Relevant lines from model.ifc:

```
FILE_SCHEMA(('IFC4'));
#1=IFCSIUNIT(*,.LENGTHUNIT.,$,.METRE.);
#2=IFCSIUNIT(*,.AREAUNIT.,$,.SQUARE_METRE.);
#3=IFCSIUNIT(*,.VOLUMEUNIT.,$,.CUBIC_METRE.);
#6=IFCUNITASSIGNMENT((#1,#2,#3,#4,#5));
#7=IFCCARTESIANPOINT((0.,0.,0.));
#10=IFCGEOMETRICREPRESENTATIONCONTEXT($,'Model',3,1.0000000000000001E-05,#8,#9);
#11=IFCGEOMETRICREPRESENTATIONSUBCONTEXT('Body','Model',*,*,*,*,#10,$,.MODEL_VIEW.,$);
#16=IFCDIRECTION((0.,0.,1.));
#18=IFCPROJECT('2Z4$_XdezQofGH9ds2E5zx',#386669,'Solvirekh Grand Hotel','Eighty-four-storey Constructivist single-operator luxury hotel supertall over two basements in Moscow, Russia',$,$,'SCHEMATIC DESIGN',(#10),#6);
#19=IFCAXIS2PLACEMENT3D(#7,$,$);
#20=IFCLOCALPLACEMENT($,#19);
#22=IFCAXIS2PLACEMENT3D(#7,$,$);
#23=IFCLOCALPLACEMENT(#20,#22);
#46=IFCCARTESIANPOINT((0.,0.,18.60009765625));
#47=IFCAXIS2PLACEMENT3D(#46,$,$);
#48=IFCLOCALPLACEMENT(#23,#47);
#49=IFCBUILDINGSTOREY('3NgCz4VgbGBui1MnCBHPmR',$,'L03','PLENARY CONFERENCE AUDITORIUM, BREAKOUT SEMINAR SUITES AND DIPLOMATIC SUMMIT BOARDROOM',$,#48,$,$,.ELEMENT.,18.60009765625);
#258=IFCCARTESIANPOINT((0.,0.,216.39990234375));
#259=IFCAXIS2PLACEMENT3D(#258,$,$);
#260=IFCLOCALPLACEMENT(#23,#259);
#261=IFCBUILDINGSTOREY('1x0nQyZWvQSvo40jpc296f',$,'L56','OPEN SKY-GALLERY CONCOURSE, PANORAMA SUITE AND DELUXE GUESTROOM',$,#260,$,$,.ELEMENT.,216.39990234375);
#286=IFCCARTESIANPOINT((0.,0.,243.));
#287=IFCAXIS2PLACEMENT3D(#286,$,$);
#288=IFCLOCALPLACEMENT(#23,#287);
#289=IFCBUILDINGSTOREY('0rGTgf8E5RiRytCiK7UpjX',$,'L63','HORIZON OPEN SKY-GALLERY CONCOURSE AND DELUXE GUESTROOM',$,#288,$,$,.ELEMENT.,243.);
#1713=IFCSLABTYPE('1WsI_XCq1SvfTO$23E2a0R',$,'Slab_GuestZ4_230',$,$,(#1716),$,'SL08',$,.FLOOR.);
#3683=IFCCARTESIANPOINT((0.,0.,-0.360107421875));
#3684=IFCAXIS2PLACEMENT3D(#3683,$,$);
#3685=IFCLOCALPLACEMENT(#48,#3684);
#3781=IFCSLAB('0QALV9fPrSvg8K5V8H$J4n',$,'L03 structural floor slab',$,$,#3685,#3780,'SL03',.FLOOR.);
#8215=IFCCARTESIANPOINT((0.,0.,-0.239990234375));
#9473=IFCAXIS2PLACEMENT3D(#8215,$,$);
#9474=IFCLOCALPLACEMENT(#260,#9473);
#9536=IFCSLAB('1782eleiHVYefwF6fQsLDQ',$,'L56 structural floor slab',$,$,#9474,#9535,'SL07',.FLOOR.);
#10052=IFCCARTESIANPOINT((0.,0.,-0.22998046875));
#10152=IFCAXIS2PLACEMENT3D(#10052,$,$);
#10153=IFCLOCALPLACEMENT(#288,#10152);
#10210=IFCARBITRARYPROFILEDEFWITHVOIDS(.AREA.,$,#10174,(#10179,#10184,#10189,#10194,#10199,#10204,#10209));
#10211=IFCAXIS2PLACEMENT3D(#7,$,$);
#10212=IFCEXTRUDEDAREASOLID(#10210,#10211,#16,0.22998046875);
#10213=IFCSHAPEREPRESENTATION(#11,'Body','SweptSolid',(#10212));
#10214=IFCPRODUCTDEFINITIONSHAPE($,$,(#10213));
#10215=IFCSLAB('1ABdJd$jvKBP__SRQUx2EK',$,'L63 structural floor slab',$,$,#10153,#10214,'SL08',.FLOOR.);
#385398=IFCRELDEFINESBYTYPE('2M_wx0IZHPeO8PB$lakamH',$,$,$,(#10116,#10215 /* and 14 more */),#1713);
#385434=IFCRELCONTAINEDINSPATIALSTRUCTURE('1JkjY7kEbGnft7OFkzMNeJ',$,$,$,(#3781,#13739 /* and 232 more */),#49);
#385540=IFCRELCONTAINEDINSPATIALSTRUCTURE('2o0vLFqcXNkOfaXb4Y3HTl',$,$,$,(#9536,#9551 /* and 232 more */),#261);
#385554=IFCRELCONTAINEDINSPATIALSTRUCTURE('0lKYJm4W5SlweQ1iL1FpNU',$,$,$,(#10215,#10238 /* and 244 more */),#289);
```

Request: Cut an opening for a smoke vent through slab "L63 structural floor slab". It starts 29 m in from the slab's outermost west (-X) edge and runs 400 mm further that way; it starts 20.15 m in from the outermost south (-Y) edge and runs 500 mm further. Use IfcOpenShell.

```python
import numpy as np
import ifcopenshell
import ifcopenshell.api.feature
import ifcopenshell.api.geometry
import ifcopenshell.api.root
import ifcopenshell.geom
import ifcopenshell.util.placement
import ifcopenshell.util.representation
import ifcopenshell.util.shape
import ifcopenshell.util.unit

model = ifcopenshell.open("model.ifc")
unit_scale = ifcopenshell.util.unit.calculate_unit_scale(model)
settings = ifcopenshell.geom.settings()


def volume(element):
    """Net volume in cubic metres, openings subtracted."""
    shape = ifcopenshell.geom.create_shape(settings, element)
    return ifcopenshell.util.shape.get_volume(shape.geometry)


slab = model.by_id(10215)
before = volume(slab)

# Extent in the slab's own axes, in metres. The edges named are its -X and -Y sides.
slab_shape = ifcopenshell.geom.create_shape(settings, slab)
vertices = ifcopenshell.util.shape.get_vertices(slab_shape.geometry)
x_min, y_min, bottom = vertices.min(axis=0)
top = vertices[:, 2].max()

opening = ifcopenshell.api.root.create_entity(model, ifc_class="IfcOpeningElement", name="Smoke vent opening", predefined_type="OPENING")
context = ifcopenshell.util.representation.get_context(model, "Model", "Body", "MODEL_VIEW")
width, depth = 0.4, 0.5
outline = [(0.0, 0.0), (width, 0.0), (width, depth), (0.0, depth), (0.0, 0.0)]
# Overshoot both faces by 50 mm so the cut is clean.
shape = ifcopenshell.api.geometry.add_slab_representation(
    model, context=context, depth=top - bottom + 0.1, polyline=outline
)
ifcopenshell.api.geometry.assign_representation(model, product=opening, representation=shape)

matrix = ifcopenshell.util.placement.get_local_placement(slab.ObjectPlacement)
matrix[:, 3] = matrix @ np.append(np.array([x_min + 29, y_min + 20.15, bottom - 0.05]) / unit_scale, 1.0)
ifcopenshell.api.geometry.edit_object_placement(model, product=opening, matrix=matrix, is_si=False)
ifcopenshell.api.feature.add_feature(model, feature=opening, element=slab)

after = volume(slab)

print(f"slab volume {before:.3f} -> {after:.3f} m3")

model.write("model_rev.ifc")
```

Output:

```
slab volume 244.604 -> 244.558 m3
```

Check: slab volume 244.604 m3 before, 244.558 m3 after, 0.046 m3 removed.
